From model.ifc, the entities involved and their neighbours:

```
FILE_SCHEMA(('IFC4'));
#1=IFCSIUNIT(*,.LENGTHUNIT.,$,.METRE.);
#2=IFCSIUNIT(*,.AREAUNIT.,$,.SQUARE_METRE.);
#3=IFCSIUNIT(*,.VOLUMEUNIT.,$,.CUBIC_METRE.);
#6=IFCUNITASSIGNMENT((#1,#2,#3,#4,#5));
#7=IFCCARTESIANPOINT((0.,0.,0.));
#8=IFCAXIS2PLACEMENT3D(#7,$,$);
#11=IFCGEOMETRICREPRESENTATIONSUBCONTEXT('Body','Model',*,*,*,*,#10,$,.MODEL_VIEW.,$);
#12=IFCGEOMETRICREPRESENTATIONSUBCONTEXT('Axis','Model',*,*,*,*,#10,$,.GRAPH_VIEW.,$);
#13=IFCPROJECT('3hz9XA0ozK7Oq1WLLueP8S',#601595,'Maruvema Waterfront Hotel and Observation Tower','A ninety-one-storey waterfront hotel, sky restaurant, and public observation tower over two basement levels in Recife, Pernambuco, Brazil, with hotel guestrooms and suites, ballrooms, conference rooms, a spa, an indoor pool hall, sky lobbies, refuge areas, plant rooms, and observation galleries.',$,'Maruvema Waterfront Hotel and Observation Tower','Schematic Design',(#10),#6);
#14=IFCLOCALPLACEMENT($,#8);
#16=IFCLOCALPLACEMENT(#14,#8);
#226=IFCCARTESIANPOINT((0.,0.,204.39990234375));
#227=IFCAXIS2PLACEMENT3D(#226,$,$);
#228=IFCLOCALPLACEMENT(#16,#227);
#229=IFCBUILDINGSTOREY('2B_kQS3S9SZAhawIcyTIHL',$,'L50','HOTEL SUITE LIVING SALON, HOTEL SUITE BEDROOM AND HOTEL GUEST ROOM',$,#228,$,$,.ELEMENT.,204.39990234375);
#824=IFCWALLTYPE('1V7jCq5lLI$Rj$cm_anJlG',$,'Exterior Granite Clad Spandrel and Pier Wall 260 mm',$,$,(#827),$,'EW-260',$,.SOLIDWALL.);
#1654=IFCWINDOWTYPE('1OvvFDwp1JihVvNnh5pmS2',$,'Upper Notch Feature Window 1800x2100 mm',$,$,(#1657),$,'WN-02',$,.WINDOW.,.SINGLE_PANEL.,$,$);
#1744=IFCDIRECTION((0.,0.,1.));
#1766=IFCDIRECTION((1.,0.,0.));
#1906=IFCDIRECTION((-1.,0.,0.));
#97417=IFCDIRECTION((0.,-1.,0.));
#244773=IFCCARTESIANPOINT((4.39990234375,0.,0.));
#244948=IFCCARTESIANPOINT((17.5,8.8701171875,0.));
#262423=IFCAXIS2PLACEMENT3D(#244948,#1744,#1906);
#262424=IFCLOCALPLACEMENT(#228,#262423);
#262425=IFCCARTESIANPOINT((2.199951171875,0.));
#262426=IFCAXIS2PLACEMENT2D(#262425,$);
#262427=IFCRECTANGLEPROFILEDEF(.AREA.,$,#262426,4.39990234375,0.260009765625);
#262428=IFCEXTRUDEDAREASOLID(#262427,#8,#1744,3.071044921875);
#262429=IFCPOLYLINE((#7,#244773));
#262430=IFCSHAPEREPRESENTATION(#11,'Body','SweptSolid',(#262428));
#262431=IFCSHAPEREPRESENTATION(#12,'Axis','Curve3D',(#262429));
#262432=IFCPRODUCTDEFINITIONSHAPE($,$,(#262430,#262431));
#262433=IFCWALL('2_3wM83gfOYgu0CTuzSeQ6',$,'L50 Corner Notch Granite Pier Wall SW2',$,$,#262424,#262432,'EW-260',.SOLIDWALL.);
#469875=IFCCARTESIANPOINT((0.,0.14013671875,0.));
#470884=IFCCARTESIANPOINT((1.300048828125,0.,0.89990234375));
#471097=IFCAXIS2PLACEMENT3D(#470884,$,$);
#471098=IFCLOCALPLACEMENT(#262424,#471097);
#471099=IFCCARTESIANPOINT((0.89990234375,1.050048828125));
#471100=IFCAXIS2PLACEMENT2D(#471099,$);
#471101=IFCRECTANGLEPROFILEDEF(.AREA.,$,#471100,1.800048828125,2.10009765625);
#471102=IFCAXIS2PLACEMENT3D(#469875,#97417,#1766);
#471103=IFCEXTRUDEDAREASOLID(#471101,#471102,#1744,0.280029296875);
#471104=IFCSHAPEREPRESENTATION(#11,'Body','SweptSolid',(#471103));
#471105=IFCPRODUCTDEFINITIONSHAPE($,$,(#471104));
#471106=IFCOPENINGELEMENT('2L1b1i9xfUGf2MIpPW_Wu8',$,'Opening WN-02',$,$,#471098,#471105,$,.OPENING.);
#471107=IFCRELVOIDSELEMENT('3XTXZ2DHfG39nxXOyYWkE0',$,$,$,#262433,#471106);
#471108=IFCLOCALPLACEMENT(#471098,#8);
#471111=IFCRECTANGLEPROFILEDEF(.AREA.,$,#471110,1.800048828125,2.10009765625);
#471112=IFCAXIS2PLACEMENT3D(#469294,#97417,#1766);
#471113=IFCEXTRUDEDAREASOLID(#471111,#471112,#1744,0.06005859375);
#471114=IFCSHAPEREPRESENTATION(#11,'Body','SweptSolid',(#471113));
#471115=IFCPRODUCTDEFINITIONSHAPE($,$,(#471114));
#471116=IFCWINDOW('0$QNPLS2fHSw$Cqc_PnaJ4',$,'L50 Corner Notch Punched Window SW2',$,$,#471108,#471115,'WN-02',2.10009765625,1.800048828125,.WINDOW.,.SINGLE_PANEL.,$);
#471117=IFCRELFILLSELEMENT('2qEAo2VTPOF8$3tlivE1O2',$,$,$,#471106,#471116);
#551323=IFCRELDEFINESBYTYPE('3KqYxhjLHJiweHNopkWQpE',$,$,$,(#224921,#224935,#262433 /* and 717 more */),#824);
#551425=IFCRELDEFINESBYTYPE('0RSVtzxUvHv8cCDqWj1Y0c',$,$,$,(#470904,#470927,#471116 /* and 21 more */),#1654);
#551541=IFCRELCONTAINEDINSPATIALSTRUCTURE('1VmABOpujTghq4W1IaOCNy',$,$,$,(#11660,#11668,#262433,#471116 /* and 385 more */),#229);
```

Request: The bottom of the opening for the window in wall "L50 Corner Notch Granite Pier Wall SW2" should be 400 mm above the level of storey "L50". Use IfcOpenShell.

```python
import numpy as np
import ifcopenshell
import ifcopenshell.api.geometry
import ifcopenshell.geom
import ifcopenshell.util.element
import ifcopenshell.util.placement
import ifcopenshell.util.shape
import ifcopenshell.util.unit

model = ifcopenshell.open("model.ifc")
unit_scale = ifcopenshell.util.unit.calculate_unit_scale(model)

window = model.by_guid("0$QNPLS2fHSw$Cqc_PnaJ4")
opening = window.FillsVoids[0].RelatingOpeningElement
storey = ifcopenshell.util.element.get_container(window, ifc_class="IfcBuildingStorey")
level = ifcopenshell.util.placement.get_local_placement(storey.ObjectPlacement)[2, 3]

# The opening's origin need not be at the sill, so measure its lowest point.
shape = ifcopenshell.geom.create_shape(ifcopenshell.geom.settings(), opening)
bottom = ifcopenshell.util.shape.get_shape_bottom_elevation(shape, shape.geometry) / unit_scale
dz = level + 0.4 - bottom

shift = np.array([0.0, 0.0, dz])
# The window is placed relative to its opening, so it follows when the opening moves.
matrix = ifcopenshell.util.placement.get_local_placement(opening.ObjectPlacement)
matrix[:3, 3] += shift
ifcopenshell.api.geometry.edit_object_placement(
    model, product=opening, matrix=matrix, is_si=False, should_transform_children=True
)

print(f"moved by {dz * unit_scale:+.3f} m")

model.write("model_rev.ifc")
```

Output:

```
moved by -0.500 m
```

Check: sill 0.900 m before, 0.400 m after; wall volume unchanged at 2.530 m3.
